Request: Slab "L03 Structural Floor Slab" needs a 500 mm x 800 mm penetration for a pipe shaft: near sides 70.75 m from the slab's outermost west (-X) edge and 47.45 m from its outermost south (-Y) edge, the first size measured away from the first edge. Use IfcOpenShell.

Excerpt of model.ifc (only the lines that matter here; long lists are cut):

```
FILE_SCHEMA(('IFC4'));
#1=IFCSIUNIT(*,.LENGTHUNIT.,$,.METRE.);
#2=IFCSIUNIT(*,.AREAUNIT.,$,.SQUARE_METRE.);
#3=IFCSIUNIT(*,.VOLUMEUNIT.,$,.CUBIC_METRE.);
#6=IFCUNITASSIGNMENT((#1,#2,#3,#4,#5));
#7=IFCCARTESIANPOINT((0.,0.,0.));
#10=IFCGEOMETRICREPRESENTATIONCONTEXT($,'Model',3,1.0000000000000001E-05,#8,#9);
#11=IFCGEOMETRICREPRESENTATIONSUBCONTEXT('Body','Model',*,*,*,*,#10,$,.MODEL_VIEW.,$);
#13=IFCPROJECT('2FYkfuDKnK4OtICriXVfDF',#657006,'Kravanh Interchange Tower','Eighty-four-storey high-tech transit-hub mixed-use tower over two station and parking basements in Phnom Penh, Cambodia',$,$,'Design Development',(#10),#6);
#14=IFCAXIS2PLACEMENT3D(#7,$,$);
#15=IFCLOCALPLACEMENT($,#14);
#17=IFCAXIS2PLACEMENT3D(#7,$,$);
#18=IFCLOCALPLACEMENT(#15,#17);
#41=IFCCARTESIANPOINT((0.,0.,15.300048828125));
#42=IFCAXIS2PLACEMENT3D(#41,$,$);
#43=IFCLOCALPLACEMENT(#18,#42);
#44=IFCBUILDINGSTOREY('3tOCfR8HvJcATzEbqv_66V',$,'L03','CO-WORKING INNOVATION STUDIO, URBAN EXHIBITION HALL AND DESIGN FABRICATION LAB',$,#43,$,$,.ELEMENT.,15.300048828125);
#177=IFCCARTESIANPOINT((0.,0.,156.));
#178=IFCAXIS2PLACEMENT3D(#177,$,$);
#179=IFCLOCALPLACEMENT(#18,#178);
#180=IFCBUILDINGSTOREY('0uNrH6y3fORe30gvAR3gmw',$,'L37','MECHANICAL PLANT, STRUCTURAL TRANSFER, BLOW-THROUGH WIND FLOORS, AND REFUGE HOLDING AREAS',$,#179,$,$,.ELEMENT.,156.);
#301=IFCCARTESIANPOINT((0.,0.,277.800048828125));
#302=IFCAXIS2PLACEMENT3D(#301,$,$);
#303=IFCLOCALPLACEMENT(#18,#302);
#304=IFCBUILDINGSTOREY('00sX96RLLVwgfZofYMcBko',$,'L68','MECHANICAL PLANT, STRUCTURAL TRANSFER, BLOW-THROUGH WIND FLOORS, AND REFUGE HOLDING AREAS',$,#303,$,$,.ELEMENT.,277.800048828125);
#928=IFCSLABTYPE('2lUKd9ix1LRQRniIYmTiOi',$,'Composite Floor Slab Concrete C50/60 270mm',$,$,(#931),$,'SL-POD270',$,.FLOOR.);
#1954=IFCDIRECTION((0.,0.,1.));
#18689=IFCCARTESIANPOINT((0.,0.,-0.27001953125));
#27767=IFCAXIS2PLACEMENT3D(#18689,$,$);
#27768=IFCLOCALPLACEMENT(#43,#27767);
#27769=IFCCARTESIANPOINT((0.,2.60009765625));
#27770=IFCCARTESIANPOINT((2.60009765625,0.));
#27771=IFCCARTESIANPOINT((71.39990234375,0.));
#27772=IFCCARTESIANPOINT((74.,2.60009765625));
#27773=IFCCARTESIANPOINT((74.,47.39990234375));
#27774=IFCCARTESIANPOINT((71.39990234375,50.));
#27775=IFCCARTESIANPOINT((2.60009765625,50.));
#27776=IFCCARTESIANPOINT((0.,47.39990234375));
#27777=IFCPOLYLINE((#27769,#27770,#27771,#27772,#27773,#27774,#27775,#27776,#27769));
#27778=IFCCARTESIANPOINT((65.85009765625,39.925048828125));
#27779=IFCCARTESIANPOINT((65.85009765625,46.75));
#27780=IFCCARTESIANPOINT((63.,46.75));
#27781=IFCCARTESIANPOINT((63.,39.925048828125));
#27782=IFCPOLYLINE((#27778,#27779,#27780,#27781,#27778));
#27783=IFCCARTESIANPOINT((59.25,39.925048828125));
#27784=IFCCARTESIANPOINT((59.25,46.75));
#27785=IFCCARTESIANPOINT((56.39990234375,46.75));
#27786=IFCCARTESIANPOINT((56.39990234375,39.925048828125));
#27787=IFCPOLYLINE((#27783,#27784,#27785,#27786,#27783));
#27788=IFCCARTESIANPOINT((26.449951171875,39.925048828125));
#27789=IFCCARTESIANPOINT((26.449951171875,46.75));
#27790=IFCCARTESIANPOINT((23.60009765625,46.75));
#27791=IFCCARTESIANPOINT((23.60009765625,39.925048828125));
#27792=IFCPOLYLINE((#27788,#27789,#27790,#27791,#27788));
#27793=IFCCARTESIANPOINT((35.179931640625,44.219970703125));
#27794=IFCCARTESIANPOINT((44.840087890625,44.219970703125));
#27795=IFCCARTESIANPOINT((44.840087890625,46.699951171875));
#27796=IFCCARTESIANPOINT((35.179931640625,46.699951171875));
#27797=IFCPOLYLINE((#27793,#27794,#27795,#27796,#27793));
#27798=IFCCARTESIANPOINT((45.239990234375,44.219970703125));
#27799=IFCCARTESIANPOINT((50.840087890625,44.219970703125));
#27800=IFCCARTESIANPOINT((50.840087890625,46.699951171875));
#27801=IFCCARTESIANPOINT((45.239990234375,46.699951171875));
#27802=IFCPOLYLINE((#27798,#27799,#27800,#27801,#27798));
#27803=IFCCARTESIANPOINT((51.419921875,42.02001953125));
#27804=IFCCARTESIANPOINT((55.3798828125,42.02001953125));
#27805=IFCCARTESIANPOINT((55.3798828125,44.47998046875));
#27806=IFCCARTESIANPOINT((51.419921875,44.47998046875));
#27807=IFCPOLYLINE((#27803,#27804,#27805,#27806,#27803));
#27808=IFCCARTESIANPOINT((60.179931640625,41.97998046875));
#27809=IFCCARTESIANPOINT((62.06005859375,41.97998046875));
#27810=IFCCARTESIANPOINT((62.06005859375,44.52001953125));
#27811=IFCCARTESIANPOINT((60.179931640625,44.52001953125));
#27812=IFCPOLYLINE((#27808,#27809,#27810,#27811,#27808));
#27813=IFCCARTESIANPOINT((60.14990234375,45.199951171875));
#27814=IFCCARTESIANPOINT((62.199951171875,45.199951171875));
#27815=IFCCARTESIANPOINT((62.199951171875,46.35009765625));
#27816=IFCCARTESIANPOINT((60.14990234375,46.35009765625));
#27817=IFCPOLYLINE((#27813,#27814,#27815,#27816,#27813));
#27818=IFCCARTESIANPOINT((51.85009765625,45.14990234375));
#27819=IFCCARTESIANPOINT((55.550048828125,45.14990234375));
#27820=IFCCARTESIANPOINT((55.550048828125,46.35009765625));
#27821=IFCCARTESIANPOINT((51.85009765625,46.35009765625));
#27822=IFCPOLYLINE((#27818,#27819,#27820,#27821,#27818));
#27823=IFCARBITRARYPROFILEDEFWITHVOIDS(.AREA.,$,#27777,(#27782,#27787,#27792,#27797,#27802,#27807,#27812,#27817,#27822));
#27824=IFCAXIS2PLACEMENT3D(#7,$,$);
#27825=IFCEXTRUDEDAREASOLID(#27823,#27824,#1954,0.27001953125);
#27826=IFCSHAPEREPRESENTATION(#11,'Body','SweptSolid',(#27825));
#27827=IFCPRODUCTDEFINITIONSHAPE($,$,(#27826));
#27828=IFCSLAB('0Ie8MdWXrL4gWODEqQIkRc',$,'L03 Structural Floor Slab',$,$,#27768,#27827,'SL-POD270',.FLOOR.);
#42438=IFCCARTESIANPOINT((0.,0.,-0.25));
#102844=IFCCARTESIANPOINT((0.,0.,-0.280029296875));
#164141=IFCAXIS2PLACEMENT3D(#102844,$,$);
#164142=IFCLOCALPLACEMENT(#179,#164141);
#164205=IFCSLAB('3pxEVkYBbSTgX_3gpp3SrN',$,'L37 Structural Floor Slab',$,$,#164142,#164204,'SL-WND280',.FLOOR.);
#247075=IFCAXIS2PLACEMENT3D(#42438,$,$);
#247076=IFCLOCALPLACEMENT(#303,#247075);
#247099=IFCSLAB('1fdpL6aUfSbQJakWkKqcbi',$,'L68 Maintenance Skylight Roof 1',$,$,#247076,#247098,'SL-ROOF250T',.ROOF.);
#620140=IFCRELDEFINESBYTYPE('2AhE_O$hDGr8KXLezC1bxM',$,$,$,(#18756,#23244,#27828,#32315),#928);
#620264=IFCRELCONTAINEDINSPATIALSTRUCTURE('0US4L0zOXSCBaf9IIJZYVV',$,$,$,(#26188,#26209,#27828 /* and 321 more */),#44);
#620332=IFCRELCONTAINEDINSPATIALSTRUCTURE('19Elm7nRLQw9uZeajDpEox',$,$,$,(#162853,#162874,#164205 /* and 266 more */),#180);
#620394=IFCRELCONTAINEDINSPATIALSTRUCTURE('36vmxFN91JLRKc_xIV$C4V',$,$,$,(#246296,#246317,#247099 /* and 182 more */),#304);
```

```python
import numpy as np
import ifcopenshell
import ifcopenshell.api.feature
import ifcopenshell.api.geometry
import ifcopenshell.api.root
import ifcopenshell.geom
import ifcopenshell.util.placement
import ifcopenshell.util.representation
import ifcopenshell.util.shape
import ifcopenshell.util.unit

model = ifcopenshell.open("model.ifc")
unit_scale = ifcopenshell.util.unit.calculate_unit_scale(model)
settings = ifcopenshell.geom.settings()


def volume(element):
    """Net volume in cubic metres, openings subtracted."""
    shape = ifcopenshell.geom.create_shape(settings, element)
    return ifcopenshell.util.shape.get_volume(shape.geometry)


slab = model.by_id(27828)
before = volume(slab)

# Extent in the slab's own axes, in metres. The edges named are its -X and -Y sides.
slab_shape = ifcopenshell.geom.create_shape(settings, slab)
vertices = ifcopenshell.util.shape.get_vertices(slab_shape.geometry)
x_min, y_min, bottom = vertices.min(axis=0)
top = vertices[:, 2].max()

opening = ifcopenshell.api.root.create_entity(model, ifc_class="IfcOpeningElement", name="Pipe shaft opening", predefined_type="OPENING")
context = ifcopenshell.util.representation.get_context(model, "Model", "Body", "MODEL_VIEW")
width, depth = 0.5, 0.8
outline = [(0.0, 0.0), (width, 0.0), (width, depth), (0.0, depth), (0.0, 0.0)]
# Overshoot both faces by 50 mm so the cut is clean.
shape = ifcopenshell.api.geometry.add_slab_representation(
    model, context=context, depth=top - bottom + 0.1, polyline=outline
)
ifcopenshell.api.geometry.assign_representation(model, product=opening, representation=shape)

matrix = ifcopenshell.util.placement.get_local_placement(slab.ObjectPlacement)
matrix[:, 3] = matrix @ np.append(np.array([x_min + 70.75, y_min + 47.45, bottom - 0.05]) / unit_scale, 1.0)
ifcopenshell.api.geometry.edit_object_placement(model, product=opening, matrix=matrix, is_si=False)
ifcopenshell.api.feature.add_feature(model, feature=opening, element=slab)

after = volume(slab)

print(f"slab volume {before:.3f} -> {after:.3f} m3")

model.write("model_rev.ifc")
```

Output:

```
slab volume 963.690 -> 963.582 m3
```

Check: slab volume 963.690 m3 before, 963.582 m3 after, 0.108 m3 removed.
